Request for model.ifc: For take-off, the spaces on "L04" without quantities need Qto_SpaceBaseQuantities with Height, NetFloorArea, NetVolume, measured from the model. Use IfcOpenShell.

First a look at what the model holds.

```python
import ifcopenshell
import ifcopenshell.util.element
import ifcopenshell.util.unit

model = ifcopenshell.open("model.ifc")
print(model.schema)
for unit_type in ("LENGTHUNIT", "AREAUNIT", "VOLUMEUNIT"):
    print(unit_type, ifcopenshell.util.unit.calculate_unit_scale(model, unit_type))
storey = next(s for s in model.by_type("IfcBuildingStorey") if s.Name == "L04")
spaces = [e for e in ifcopenshell.util.element.get_decomposition(storey) if e.is_a("IfcSpace")]
for e in sorted(spaces, key=lambda e: e.id()):
    print(e.id(), e.is_a(), e.Name, list(ifcopenshell.util.element.get_psets(e, qtos_only=True)), sep=" | ")
```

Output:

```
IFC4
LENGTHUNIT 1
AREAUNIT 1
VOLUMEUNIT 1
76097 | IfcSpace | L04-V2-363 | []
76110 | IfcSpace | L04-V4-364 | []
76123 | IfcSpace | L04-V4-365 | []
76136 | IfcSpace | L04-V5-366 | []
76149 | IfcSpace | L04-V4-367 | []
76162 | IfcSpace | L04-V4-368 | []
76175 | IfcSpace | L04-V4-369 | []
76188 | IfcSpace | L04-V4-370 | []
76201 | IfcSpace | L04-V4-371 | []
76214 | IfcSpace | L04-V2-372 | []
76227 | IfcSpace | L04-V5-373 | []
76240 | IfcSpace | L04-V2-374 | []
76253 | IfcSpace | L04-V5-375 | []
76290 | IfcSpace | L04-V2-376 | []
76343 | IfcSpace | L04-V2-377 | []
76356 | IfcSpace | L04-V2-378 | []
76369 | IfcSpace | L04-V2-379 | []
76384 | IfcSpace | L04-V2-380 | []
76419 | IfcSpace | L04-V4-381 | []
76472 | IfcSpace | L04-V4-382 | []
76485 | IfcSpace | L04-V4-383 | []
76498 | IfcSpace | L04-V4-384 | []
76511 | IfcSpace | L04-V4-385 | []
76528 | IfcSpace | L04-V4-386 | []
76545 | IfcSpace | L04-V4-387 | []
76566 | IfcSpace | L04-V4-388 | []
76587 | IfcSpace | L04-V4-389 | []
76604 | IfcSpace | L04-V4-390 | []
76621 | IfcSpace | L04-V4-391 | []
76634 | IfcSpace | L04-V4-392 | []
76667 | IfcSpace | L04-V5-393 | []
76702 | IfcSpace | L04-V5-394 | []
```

```python
import ifcopenshell
import ifcopenshell.api.pset
import ifcopenshell.geom
import ifcopenshell.util.element
import ifcopenshell.util.shape
import ifcopenshell.util.unit

model = ifcopenshell.open("model.ifc")
unit_scale = ifcopenshell.util.unit.calculate_unit_scale(model)
area_scale = ifcopenshell.util.unit.calculate_unit_scale(model, "AREAUNIT")
volume_scale = ifcopenshell.util.unit.calculate_unit_scale(model, "VOLUMEUNIT")
settings = ifcopenshell.geom.settings()

storey = next(s for s in model.by_type("IfcBuildingStorey") if s.Name == "L04")
spaces = [e for e in ifcopenshell.util.element.get_decomposition(storey) if e.is_a("IfcSpace")]

for e in sorted(spaces, key=lambda e: e.id()):
    if ifcopenshell.util.element.get_psets(e, qtos_only=True, should_inherit=False):
        continue
    # Geometry comes back in metres, in the element's own axes.
    shape = ifcopenshell.geom.create_shape(settings, e)
    values = {
        "Height": ifcopenshell.util.shape.get_z(shape.geometry) / unit_scale,
        "NetFloorArea": ifcopenshell.util.shape.get_footprint_area(shape.geometry) / area_scale,
        "NetVolume": ifcopenshell.util.shape.get_volume(shape.geometry) / volume_scale,
    }
    qto = ifcopenshell.api.pset.add_qto(model, product=e, name="Qto_SpaceBaseQuantities")
    ifcopenshell.api.pset.edit_qto(model, qto=qto, properties=values)
    print(e.id(), {k: round(v, 3) for k, v in values.items()})

model.write("model_updated.ifc")
```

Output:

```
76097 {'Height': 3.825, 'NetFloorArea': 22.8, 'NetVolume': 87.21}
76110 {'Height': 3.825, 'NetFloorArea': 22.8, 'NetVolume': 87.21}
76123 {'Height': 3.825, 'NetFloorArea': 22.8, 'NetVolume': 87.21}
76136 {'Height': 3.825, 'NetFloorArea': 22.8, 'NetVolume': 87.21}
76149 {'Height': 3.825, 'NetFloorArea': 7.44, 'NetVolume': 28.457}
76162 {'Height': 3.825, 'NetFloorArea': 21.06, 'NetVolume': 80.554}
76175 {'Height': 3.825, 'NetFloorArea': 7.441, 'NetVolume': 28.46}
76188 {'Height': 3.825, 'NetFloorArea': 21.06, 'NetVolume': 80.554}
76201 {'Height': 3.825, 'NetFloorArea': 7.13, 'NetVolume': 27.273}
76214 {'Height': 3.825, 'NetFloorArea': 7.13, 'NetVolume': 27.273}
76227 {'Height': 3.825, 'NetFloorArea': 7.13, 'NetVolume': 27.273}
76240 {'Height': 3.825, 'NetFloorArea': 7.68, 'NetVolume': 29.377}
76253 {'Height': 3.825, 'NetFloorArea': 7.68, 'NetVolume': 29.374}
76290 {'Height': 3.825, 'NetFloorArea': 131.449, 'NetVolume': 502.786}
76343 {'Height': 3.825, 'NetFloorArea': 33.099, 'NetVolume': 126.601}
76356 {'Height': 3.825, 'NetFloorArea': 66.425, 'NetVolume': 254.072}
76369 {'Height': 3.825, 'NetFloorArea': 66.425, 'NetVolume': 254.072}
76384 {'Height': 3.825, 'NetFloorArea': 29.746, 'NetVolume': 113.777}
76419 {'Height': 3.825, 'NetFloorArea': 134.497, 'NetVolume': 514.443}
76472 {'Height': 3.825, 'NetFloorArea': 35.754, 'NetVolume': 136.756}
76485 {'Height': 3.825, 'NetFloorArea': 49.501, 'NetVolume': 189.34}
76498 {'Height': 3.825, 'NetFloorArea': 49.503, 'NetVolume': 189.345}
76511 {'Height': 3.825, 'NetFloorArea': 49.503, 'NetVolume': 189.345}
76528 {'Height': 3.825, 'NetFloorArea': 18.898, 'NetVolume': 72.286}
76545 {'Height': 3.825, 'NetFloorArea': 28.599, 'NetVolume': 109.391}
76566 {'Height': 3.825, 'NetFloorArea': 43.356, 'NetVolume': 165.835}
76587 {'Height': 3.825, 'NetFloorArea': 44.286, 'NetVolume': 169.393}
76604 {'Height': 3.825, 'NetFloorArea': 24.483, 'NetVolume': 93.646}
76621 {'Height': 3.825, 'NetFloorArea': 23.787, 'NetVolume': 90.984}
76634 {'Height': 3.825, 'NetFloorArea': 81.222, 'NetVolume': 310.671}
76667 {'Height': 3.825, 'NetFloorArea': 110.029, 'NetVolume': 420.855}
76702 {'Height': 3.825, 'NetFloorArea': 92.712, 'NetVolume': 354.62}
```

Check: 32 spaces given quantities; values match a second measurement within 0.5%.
